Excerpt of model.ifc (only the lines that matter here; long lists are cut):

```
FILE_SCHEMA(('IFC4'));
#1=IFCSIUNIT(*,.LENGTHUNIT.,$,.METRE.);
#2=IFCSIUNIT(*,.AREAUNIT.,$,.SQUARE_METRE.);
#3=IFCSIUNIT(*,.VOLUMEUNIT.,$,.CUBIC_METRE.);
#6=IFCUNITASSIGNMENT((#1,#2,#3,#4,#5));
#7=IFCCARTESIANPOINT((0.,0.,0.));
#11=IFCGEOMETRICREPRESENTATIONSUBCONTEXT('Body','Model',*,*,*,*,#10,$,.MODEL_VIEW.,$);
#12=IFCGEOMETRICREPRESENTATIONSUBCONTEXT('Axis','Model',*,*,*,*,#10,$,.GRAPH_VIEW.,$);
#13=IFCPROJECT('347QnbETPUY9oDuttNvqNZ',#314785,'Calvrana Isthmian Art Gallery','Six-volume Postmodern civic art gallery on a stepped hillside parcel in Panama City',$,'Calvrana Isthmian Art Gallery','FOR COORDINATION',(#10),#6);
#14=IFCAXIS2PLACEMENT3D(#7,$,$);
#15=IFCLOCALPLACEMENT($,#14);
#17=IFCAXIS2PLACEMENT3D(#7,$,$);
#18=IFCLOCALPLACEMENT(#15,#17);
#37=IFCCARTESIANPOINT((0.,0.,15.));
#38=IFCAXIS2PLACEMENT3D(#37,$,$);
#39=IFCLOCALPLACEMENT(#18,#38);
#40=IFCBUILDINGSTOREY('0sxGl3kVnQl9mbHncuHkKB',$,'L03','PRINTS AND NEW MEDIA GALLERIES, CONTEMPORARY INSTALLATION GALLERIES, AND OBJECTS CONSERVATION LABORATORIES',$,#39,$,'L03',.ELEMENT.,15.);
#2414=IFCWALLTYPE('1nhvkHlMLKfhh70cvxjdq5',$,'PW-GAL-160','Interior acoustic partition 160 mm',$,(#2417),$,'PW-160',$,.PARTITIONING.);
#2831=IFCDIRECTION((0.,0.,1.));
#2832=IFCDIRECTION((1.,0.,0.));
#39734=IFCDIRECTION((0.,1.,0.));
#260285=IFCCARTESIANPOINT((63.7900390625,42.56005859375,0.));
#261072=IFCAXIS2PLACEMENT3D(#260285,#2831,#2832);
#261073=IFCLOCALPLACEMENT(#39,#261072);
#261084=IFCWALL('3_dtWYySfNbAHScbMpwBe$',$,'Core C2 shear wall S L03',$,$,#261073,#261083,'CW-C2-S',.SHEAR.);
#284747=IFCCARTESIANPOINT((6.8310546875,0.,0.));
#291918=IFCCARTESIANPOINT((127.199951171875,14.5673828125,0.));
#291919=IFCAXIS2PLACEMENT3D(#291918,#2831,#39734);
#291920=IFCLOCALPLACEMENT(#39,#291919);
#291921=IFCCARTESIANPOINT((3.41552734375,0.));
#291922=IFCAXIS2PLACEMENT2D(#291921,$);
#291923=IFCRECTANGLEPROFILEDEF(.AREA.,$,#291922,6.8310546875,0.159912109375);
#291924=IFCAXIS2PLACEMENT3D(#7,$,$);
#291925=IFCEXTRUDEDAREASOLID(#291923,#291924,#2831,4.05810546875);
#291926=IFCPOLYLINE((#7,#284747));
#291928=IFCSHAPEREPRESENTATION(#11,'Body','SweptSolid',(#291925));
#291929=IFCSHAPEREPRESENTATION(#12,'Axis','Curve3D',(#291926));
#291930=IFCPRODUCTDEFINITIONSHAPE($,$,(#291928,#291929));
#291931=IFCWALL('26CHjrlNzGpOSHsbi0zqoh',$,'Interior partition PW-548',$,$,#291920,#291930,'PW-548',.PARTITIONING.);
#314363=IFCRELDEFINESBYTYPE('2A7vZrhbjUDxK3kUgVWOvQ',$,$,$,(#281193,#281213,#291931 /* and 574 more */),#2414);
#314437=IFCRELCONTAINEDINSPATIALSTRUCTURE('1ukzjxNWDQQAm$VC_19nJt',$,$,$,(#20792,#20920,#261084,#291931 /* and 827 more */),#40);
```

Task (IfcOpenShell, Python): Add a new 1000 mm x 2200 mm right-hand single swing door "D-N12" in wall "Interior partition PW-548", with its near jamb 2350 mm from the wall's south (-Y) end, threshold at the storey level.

```python
import numpy as np
import ifcopenshell
import ifcopenshell.api.feature
import ifcopenshell.api.geometry
import ifcopenshell.api.root
import ifcopenshell.api.spatial
import ifcopenshell.geom
import ifcopenshell.util.element
import ifcopenshell.util.placement
import ifcopenshell.util.representation
import ifcopenshell.util.shape
import ifcopenshell.util.unit

model = ifcopenshell.open("model.ifc")
unit_scale = ifcopenshell.util.unit.calculate_unit_scale(model)
settings = ifcopenshell.geom.settings()


def volume(element):
    """Net volume in cubic metres, openings subtracted."""
    shape = ifcopenshell.geom.create_shape(settings, element)
    return ifcopenshell.util.shape.get_volume(shape.geometry)


wall = model.by_guid("26CHjrlNzGpOSHsbi0zqoh")
storey = ifcopenshell.util.element.get_container(wall, ifc_class="IfcBuildingStorey")
context = ifcopenshell.util.representation.get_context(model, "Model", "Body", "MODEL_VIEW")
before = volume(wall)

width, height, from_end, sill = 1, 2.2, 2.35, 0.0  # metres

# The wall runs along its own X axis, and the end named is its -X end.
wall_shape = ifcopenshell.geom.create_shape(settings, wall)
x, y, z = ifcopenshell.util.shape.get_vertices(wall_shape.geometry).T
start = x.min() + from_end
face, thickness = float(y.min()), float(y.max() - y.min())
wall_matrix = ifcopenshell.util.placement.get_local_placement(wall.ObjectPlacement)
level = ifcopenshell.util.placement.get_local_placement(storey.ObjectPlacement)[2, 3]


def in_wall(x, y):
    """Placement at x, y metres in the wall's axes, at sill height."""
    matrix = wall_matrix.copy()
    matrix[:, 3] = wall_matrix @ np.array([x / unit_scale, y / unit_scale, 0.0, 1.0])
    matrix[2, 3] = level + sill / unit_scale
    return matrix


# Opening: a box that overshoots both wall faces by 50 mm.
opening = ifcopenshell.api.root.create_entity(model, ifc_class="IfcOpeningElement", predefined_type="OPENING")
box = ifcopenshell.api.geometry.add_wall_representation(
    model, context=context, length=width, height=height, thickness=thickness + 0.1
)
ifcopenshell.api.geometry.assign_representation(model, product=opening, representation=box)
ifcopenshell.api.geometry.edit_object_placement(model, product=opening, matrix=in_wall(start, face - 0.05), is_si=False)
ifcopenshell.api.feature.add_feature(model, feature=opening, element=wall)

door = ifcopenshell.api.root.create_entity(model, ifc_class="IfcDoor", name="D-N12", predefined_type="DOOR")
door.OverallWidth, door.OverallHeight = width / unit_scale, height / unit_scale
door.OperationType = "SINGLE_SWING_RIGHT"
body = ifcopenshell.api.geometry.add_door_representation(
    model,
    context=context,
    overall_width=door.OverallWidth,
    overall_height=door.OverallHeight,
    operation_type="SINGLE_SWING_RIGHT",
    lining_properties={"LiningDepth": thickness / unit_scale, "ThresholdDepth": thickness / unit_scale},
)
ifcopenshell.api.geometry.assign_representation(model, product=door, representation=body)
ifcopenshell.api.spatial.assign_container(model, products=[door], relating_structure=storey)
ifcopenshell.api.feature.add_filling(model, opening=opening, element=door)

# The lining spans the wall, so the door starts at the wall face.
ifcopenshell.api.geometry.edit_object_placement(model, product=door, matrix=in_wall(start, face), is_si=False)

after = volume(wall)

print(f"wall volume {before:.3f} -> {after:.3f} m3")

model.write("model-out.ifc")
```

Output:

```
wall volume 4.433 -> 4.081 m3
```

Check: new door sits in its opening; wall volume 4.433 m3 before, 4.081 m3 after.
